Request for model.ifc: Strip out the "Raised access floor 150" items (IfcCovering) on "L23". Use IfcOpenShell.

First a look at what the model holds.

```python
import ifcopenshell
import ifcopenshell.util.element

model = ifcopenshell.open("model.ifc")
print(model.schema)
storey = next(s for s in model.by_type("IfcBuildingStorey") if s.Name == "L23")
coverings = [e for e in ifcopenshell.util.element.get_decomposition(storey) if e.is_a("IfcCovering")]
seen = {}
for e in coverings:
    element_type = ifcopenshell.util.element.get_type(e)
    name = element_type.Name if element_type not in (None, e) else None
    seen[name] = seen.get(name, 0) + 1
for name, count in sorted(seen.items(), key=str):
    print(count, "x", name)
```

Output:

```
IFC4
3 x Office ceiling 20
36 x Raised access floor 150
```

```python
import ifcopenshell
import ifcopenshell.api.root
import ifcopenshell.util.element

model = ifcopenshell.open("model.ifc")

storey = next(s for s in model.by_type("IfcBuildingStorey") if s.Name == "L23")
coverings = [e for e in ifcopenshell.util.element.get_decomposition(storey) if e.is_a("IfcCovering")]
targets = [e for e in coverings if (t := ifcopenshell.util.element.get_type(e)) not in (None, e) and t.Name == "Raised access floor 150"]

for e in targets:
    ifcopenshell.api.root.remove_product(model, product=e)
print(len(targets), "removed")

model.write("model_updated.ifc")
```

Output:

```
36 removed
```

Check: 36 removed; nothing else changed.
